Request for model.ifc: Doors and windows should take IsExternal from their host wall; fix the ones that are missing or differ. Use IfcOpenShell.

First a look at what the model holds.

```python
import ifcopenshell
import ifcopenshell.util.element

model = ifcopenshell.open("model.ifc")
print(model.schema)
seen = {}
for e in model.by_type("IfcDoor") + model.by_type("IfcWindow"):
    if not e.FillsVoids:
        continue
    host = e.FillsVoids[0].RelatingOpeningElement.VoidsElements[0].RelatingBuildingElement
    own = ifcopenshell.util.element.get_pset(e, f"Pset_{e.is_a()[3:].removesuffix('StandardCase')}Common", "IsExternal")
    wall = ifcopenshell.util.element.get_pset(host, "Pset_WallCommon", "IsExternal")
    seen[e.is_a(), own, wall] = seen.get((e.is_a(), own, wall), 0) + 1
for (cls, own, wall), count in sorted(seen.items(), key=str):
    print(count, cls, "IsExternal:", own, "| host wall:", wall)
```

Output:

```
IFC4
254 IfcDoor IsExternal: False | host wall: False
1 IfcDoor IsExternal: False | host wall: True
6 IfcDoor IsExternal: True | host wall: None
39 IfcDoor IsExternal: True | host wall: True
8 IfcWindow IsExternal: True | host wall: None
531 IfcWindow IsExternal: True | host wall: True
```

```python
import ifcopenshell
import ifcopenshell.api.pset
import ifcopenshell.util.element

model = ifcopenshell.open("model.ifc")

count = 0
for ifc_class, pset_name in (("IfcDoor", "Pset_DoorCommon"), ("IfcWindow", "Pset_WindowCommon")):
    for e in model.by_type(ifc_class):
        if not e.FillsVoids:
            continue
        host = e.FillsVoids[0].RelatingOpeningElement.VoidsElements[0].RelatingBuildingElement
        external = ifcopenshell.util.element.get_pset(host, "Pset_WallCommon", "IsExternal")
        if external is None or ifcopenshell.util.element.get_pset(e, pset_name, "IsExternal") == external:
            continue
        pset = ifcopenshell.api.pset.add_pset(model, product=e, name=pset_name)
        ifcopenshell.api.pset.edit_pset(model, pset=pset, properties={"IsExternal": external})
        count += 1

print(count, "updated")

model.write("model_updated.ifc")
```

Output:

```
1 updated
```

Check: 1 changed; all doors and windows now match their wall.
